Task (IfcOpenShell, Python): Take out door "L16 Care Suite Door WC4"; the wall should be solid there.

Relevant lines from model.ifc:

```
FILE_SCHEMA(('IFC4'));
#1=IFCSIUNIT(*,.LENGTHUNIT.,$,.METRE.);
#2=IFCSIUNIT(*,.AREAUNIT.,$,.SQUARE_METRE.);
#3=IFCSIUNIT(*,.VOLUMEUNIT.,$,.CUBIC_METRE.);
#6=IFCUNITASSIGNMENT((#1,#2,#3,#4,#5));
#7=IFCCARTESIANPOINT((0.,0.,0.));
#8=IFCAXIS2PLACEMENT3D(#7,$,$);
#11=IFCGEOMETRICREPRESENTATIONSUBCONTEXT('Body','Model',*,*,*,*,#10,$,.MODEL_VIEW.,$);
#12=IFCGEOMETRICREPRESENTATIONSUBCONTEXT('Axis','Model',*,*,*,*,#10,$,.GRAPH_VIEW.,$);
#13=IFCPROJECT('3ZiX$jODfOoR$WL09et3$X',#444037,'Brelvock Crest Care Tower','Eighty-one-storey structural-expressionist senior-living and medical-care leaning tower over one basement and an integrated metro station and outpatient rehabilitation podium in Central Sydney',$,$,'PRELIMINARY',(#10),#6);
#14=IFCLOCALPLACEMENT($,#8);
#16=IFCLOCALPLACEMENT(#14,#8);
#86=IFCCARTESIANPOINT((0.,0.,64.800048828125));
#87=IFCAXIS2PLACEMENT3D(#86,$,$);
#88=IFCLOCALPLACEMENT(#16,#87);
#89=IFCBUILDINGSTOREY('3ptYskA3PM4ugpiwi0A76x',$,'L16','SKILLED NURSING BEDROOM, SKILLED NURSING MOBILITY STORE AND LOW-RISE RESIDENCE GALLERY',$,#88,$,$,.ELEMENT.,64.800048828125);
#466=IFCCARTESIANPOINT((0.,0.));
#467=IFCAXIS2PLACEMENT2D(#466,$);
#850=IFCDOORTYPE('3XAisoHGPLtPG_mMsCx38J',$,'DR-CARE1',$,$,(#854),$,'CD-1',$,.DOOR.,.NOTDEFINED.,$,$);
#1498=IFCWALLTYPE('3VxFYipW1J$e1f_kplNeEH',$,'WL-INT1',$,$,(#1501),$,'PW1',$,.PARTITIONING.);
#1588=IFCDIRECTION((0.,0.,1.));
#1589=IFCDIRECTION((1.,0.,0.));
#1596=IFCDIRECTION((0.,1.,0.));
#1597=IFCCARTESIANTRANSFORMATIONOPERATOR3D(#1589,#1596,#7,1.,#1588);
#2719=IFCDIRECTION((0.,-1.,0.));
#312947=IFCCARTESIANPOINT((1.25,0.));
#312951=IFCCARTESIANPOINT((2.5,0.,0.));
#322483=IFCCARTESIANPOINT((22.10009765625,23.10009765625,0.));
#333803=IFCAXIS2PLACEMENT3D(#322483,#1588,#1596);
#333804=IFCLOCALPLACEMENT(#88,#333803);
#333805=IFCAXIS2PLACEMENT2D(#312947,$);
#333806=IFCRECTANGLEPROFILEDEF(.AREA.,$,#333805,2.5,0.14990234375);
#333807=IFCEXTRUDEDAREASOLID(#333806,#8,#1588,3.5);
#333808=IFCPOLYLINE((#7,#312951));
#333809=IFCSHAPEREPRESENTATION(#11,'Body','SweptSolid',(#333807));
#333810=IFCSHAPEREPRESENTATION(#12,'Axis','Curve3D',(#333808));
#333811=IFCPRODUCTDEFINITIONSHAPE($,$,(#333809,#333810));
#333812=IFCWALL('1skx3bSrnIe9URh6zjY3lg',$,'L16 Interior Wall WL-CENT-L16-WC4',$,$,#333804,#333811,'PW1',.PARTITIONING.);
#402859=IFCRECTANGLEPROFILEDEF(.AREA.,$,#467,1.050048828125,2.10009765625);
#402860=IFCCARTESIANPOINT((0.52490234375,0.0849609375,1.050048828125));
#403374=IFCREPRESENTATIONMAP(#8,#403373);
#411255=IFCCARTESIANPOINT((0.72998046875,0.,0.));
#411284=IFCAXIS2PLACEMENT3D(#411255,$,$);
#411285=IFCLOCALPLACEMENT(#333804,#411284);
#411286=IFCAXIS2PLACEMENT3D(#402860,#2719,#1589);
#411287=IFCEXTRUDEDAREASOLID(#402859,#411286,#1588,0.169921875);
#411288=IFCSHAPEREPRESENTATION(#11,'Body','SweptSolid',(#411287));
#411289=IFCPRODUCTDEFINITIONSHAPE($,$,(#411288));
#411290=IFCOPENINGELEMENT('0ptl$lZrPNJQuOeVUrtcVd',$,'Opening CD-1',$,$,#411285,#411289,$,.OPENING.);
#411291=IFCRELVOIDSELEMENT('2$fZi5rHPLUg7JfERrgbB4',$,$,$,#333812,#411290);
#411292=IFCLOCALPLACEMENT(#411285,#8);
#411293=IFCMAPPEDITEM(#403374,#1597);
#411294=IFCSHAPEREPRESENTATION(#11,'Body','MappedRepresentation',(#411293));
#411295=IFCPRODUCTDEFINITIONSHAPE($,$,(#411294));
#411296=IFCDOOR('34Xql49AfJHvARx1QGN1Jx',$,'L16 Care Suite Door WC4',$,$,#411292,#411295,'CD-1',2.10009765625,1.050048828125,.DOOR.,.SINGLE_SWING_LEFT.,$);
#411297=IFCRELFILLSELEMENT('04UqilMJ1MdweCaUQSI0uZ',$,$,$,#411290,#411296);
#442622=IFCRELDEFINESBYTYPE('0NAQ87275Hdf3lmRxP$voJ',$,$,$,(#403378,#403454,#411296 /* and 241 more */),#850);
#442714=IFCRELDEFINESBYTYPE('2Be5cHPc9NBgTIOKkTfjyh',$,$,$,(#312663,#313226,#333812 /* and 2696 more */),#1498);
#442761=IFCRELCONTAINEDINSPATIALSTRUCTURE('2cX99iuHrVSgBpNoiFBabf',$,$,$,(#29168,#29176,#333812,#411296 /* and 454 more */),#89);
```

```python
import ifcopenshell
import ifcopenshell.api.feature
import ifcopenshell.api.root
import ifcopenshell.geom
import ifcopenshell.util.shape

model = ifcopenshell.open("model.ifc")
settings = ifcopenshell.geom.settings()


def volume(element):
    """Net volume in cubic metres, openings subtracted."""
    shape = ifcopenshell.geom.create_shape(settings, element)
    return ifcopenshell.util.shape.get_volume(shape.geometry)


door = model.by_guid("34Xql49AfJHvARx1QGN1Jx")
opening = door.FillsVoids[0].RelatingOpeningElement
wall = opening.VoidsElements[0].RelatingBuildingElement
before = volume(wall)

ifcopenshell.api.root.remove_product(model, product=door)
ifcopenshell.api.feature.remove_feature(model, feature=opening)

after = volume(wall)

print(f"wall volume {before:.3f} -> {after:.3f} m3")

model.write("model_edited.ifc")
```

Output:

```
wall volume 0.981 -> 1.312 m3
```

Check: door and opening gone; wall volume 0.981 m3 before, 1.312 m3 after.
